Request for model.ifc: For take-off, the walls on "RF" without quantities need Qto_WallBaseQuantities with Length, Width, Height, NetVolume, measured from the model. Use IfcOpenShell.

First a look at what the model holds.

```python
import ifcopenshell
import ifcopenshell.util.element
import ifcopenshell.util.unit

model = ifcopenshell.open("model.ifc")
print(model.schema)
for unit_type in ("LENGTHUNIT", "AREAUNIT", "VOLUMEUNIT"):
    print(unit_type, ifcopenshell.util.unit.calculate_unit_scale(model, unit_type))
storey = next(s for s in model.by_type("IfcBuildingStorey") if s.Name == "RF")
walls = [e for e in ifcopenshell.util.element.get_decomposition(storey) if e.is_a("IfcWall")]
for e in sorted(walls, key=lambda e: e.id()):
    print(e.id(), e.is_a(), e.Name, list(ifcopenshell.util.element.get_psets(e, qtos_only=True)), sep=" | ")
```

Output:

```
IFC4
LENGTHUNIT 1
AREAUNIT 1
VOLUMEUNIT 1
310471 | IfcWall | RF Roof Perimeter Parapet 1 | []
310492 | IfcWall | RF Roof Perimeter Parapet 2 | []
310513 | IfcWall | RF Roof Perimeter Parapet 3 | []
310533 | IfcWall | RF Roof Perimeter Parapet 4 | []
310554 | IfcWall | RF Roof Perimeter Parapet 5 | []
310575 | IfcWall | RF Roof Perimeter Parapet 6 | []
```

```python
import ifcopenshell
import ifcopenshell.api.pset
import ifcopenshell.geom
import ifcopenshell.util.element
import ifcopenshell.util.shape
import ifcopenshell.util.unit

model = ifcopenshell.open("model.ifc")
unit_scale = ifcopenshell.util.unit.calculate_unit_scale(model)
volume_scale = ifcopenshell.util.unit.calculate_unit_scale(model, "VOLUMEUNIT")
settings = ifcopenshell.geom.settings()

storey = next(s for s in model.by_type("IfcBuildingStorey") if s.Name == "RF")
walls = [e for e in ifcopenshell.util.element.get_decomposition(storey) if e.is_a("IfcWall")]

for e in sorted(walls, key=lambda e: e.id()):
    if ifcopenshell.util.element.get_psets(e, qtos_only=True, should_inherit=False):
        continue
    # Geometry comes back in metres, in the element's own axes.
    shape = ifcopenshell.geom.create_shape(settings, e)
    values = {
        "Length": ifcopenshell.util.shape.get_x(shape.geometry) / unit_scale,
        "Width": ifcopenshell.util.shape.get_y(shape.geometry) / unit_scale,
        "Height": ifcopenshell.util.shape.get_z(shape.geometry) / unit_scale,
        "NetVolume": ifcopenshell.util.shape.get_volume(shape.geometry) / volume_scale,
    }
    qto = ifcopenshell.api.pset.add_qto(model, product=e, name="Qto_WallBaseQuantities")
    ifcopenshell.api.pset.edit_qto(model, qto=qto, properties=values)
    print(e.id(), {k: round(v, 3) for k, v in values.items()})

model.write("model-out.ifc")
```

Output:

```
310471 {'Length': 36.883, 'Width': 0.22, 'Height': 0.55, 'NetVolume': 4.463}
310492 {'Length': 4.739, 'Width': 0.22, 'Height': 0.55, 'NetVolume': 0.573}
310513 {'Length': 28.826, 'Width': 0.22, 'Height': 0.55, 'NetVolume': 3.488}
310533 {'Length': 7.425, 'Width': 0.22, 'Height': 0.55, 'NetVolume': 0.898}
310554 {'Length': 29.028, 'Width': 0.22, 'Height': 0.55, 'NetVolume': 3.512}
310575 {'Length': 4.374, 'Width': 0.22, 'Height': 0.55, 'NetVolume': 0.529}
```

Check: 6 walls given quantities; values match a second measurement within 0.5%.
